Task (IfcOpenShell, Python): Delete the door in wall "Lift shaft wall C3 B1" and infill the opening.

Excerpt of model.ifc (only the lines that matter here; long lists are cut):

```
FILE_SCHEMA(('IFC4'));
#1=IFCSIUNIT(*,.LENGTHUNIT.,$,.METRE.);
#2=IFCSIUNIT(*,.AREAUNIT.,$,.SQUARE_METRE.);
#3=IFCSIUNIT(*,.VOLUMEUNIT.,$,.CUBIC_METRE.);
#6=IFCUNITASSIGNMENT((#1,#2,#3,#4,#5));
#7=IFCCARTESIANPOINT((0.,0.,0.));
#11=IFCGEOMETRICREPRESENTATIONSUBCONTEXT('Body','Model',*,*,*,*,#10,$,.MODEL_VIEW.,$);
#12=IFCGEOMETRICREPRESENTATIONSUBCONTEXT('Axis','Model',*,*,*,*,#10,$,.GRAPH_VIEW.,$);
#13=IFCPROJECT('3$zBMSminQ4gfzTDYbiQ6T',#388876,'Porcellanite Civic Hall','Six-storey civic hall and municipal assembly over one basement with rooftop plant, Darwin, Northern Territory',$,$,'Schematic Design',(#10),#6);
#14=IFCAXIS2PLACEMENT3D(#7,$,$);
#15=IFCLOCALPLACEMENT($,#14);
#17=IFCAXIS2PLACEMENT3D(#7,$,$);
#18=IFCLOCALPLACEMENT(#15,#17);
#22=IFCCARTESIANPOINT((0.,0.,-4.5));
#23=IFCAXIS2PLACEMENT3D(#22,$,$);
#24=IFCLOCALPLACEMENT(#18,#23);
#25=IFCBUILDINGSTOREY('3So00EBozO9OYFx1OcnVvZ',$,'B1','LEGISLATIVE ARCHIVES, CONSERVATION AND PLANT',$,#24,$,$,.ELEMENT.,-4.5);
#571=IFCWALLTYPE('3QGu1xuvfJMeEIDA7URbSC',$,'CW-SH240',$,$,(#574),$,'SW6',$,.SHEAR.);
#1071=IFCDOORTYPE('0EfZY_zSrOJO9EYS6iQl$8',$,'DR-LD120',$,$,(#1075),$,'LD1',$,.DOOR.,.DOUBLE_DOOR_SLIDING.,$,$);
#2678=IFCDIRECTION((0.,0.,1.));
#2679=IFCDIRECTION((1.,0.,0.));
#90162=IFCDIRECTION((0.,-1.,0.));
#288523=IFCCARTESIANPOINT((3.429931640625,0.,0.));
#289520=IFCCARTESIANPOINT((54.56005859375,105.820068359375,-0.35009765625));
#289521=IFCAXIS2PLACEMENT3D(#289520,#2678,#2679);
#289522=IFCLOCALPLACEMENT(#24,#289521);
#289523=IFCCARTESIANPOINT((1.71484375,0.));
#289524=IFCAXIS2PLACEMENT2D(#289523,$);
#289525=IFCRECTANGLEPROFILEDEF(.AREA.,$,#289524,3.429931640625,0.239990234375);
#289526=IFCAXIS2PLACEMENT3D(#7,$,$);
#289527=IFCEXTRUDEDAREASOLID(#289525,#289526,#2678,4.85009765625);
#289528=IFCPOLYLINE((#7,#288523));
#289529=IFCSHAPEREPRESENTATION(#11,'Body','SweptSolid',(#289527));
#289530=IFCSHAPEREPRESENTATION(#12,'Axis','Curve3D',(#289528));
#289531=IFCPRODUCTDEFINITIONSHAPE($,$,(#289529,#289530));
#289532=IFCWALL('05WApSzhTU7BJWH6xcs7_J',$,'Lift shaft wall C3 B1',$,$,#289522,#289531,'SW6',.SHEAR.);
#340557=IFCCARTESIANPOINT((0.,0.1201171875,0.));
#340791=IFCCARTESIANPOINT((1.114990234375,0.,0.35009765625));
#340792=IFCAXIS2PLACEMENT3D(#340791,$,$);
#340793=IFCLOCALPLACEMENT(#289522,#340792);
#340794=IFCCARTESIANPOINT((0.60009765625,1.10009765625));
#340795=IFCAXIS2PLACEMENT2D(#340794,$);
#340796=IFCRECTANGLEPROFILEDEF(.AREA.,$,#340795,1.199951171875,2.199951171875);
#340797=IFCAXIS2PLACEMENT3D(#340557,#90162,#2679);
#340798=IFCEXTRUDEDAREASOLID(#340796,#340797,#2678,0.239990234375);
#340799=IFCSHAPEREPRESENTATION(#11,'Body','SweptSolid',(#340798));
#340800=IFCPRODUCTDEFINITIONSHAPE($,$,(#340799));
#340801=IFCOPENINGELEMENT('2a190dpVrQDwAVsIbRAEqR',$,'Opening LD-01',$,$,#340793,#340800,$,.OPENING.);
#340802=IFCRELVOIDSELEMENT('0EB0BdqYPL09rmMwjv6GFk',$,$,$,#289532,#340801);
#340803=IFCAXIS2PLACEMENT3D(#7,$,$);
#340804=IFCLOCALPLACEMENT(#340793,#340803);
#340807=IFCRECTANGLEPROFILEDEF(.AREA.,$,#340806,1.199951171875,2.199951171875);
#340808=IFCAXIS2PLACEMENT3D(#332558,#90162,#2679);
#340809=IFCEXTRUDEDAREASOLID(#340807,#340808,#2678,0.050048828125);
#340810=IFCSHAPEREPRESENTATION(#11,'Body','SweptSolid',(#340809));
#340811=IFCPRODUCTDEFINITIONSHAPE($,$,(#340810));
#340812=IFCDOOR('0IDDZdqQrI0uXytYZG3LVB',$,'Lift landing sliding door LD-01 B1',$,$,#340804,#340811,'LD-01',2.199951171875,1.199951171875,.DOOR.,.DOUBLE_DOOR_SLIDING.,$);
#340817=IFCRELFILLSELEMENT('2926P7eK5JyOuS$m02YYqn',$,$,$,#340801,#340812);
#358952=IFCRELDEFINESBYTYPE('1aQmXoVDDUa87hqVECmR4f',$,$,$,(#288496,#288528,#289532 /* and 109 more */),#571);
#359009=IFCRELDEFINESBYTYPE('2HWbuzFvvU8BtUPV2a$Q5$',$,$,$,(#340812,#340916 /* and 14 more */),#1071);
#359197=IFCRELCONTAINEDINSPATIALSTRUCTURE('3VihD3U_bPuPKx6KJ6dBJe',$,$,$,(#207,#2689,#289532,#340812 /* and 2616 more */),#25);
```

```python
import ifcopenshell
import ifcopenshell.api.feature
import ifcopenshell.api.root
import ifcopenshell.geom
import ifcopenshell.util.shape

model = ifcopenshell.open("model.ifc")
settings = ifcopenshell.geom.settings()


def volume(element):
    """Net volume in cubic metres, openings subtracted."""
    shape = ifcopenshell.geom.create_shape(settings, element)
    return ifcopenshell.util.shape.get_volume(shape.geometry)


door = model.by_guid("0IDDZdqQrI0uXytYZG3LVB")
opening = door.FillsVoids[0].RelatingOpeningElement
wall = opening.VoidsElements[0].RelatingBuildingElement
before = volume(wall)

ifcopenshell.api.root.remove_product(model, product=door)
ifcopenshell.api.feature.remove_feature(model, feature=opening)

after = volume(wall)

print(f"wall volume {before:.3f} -> {after:.3f} m3")

model.write("model_updated.ifc")
```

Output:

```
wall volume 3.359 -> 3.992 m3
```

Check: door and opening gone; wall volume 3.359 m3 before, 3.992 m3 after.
